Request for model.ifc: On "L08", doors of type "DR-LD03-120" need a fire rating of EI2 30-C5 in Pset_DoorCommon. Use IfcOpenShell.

First a look at what the model holds.

```python
import ifcopenshell
import ifcopenshell.util.element

model = ifcopenshell.open("model.ifc")
print(model.schema)
storey = next(s for s in model.by_type("IfcBuildingStorey") if s.Name == "L08")
doors = [e for e in ifcopenshell.util.element.get_decomposition(storey) if e.is_a("IfcDoor")]
seen = {}
for e in doors:
    element_type = ifcopenshell.util.element.get_type(e)
    key = (element_type.Name if element_type != e and element_type else None, ifcopenshell.util.element.get_pset(e, "Pset_DoorCommon", "FireRating"))
    seen[key] = seen.get(key, 0) + 1
for (name, value), count in sorted(seen.items(), key=str):
    print(count, "x", name, "|", value)
```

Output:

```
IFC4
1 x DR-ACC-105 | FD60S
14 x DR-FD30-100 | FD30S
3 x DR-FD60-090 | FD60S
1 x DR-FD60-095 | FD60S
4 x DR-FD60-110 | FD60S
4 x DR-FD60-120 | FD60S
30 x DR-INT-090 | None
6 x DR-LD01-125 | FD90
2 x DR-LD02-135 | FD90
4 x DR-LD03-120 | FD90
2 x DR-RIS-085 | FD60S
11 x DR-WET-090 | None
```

```python
import ifcopenshell
import ifcopenshell.api.pset
import ifcopenshell.util.element

model = ifcopenshell.open("model.ifc")

storey = next(s for s in model.by_type("IfcBuildingStorey") if s.Name == "L08")
doors = [e for e in ifcopenshell.util.element.get_decomposition(storey) if e.is_a("IfcDoor")]

count = 0
for e in doors:
    element_type = ifcopenshell.util.element.get_type(e)
    if element_type in (None, e) or element_type.Name != "DR-LD03-120":
        continue
    found = ifcopenshell.util.element.get_pset(e, "Pset_DoorCommon", should_inherit=False)
    if found:
        pset = model.by_id(found["id"])
        if len(ifcopenshell.util.element.get_elements_by_pset(pset)) > 1:
            pset = ifcopenshell.api.pset.unshare_pset(model, products=[e], pset=pset)[0]
    else:
        pset = ifcopenshell.api.pset.add_pset(model, product=e, name="Pset_DoorCommon")
    ifcopenshell.api.pset.edit_pset(model, pset=pset, properties={"FireRating": "EI2 30-C5"})
    count += 1

print(count, "doors updated")

model.write("model_v2.ifc")
```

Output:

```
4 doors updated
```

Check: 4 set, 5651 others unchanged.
